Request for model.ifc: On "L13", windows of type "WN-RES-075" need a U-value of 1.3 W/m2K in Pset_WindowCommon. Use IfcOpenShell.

First a look at what the model holds.

```python
import ifcopenshell
import ifcopenshell.util.element

model = ifcopenshell.open("model.ifc")
print(model.schema)
storey = next(s for s in model.by_type("IfcBuildingStorey") if s.Name == "L13")
windows = [e for e in ifcopenshell.util.element.get_decomposition(storey) if e.is_a("IfcWindow")]
seen = {}
for e in windows:
    element_type = ifcopenshell.util.element.get_type(e)
    key = (element_type.Name if element_type != e and element_type else None, ifcopenshell.util.element.get_pset(e, "Pset_WindowCommon", "ThermalTransmittance"))
    seen[key] = seen.get(key, 0) + 1
for (name, value), count in sorted(seen.items(), key=str):
    print(count, "x", name, "|", value)
```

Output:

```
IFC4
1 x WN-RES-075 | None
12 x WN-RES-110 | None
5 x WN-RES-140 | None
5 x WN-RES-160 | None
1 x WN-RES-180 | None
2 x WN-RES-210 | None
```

```python
import ifcopenshell
import ifcopenshell.api.pset
import ifcopenshell.util.element

model = ifcopenshell.open("model.ifc")

storey = next(s for s in model.by_type("IfcBuildingStorey") if s.Name == "L13")
windows = [e for e in ifcopenshell.util.element.get_decomposition(storey) if e.is_a("IfcWindow")]

count = 0
for e in windows:
    element_type = ifcopenshell.util.element.get_type(e)
    if element_type in (None, e) or element_type.Name != "WN-RES-075":
        continue
    # add_pset returns the element's existing set when there is one.
    pset = ifcopenshell.api.pset.add_pset(model, product=e, name="Pset_WindowCommon")
    ifcopenshell.api.pset.edit_pset(model, pset=pset, properties={"ThermalTransmittance": 1.3})
    count += 1

print(count, "windows updated")

model.write("model_edited.ifc")
```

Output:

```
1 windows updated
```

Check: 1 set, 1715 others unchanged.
